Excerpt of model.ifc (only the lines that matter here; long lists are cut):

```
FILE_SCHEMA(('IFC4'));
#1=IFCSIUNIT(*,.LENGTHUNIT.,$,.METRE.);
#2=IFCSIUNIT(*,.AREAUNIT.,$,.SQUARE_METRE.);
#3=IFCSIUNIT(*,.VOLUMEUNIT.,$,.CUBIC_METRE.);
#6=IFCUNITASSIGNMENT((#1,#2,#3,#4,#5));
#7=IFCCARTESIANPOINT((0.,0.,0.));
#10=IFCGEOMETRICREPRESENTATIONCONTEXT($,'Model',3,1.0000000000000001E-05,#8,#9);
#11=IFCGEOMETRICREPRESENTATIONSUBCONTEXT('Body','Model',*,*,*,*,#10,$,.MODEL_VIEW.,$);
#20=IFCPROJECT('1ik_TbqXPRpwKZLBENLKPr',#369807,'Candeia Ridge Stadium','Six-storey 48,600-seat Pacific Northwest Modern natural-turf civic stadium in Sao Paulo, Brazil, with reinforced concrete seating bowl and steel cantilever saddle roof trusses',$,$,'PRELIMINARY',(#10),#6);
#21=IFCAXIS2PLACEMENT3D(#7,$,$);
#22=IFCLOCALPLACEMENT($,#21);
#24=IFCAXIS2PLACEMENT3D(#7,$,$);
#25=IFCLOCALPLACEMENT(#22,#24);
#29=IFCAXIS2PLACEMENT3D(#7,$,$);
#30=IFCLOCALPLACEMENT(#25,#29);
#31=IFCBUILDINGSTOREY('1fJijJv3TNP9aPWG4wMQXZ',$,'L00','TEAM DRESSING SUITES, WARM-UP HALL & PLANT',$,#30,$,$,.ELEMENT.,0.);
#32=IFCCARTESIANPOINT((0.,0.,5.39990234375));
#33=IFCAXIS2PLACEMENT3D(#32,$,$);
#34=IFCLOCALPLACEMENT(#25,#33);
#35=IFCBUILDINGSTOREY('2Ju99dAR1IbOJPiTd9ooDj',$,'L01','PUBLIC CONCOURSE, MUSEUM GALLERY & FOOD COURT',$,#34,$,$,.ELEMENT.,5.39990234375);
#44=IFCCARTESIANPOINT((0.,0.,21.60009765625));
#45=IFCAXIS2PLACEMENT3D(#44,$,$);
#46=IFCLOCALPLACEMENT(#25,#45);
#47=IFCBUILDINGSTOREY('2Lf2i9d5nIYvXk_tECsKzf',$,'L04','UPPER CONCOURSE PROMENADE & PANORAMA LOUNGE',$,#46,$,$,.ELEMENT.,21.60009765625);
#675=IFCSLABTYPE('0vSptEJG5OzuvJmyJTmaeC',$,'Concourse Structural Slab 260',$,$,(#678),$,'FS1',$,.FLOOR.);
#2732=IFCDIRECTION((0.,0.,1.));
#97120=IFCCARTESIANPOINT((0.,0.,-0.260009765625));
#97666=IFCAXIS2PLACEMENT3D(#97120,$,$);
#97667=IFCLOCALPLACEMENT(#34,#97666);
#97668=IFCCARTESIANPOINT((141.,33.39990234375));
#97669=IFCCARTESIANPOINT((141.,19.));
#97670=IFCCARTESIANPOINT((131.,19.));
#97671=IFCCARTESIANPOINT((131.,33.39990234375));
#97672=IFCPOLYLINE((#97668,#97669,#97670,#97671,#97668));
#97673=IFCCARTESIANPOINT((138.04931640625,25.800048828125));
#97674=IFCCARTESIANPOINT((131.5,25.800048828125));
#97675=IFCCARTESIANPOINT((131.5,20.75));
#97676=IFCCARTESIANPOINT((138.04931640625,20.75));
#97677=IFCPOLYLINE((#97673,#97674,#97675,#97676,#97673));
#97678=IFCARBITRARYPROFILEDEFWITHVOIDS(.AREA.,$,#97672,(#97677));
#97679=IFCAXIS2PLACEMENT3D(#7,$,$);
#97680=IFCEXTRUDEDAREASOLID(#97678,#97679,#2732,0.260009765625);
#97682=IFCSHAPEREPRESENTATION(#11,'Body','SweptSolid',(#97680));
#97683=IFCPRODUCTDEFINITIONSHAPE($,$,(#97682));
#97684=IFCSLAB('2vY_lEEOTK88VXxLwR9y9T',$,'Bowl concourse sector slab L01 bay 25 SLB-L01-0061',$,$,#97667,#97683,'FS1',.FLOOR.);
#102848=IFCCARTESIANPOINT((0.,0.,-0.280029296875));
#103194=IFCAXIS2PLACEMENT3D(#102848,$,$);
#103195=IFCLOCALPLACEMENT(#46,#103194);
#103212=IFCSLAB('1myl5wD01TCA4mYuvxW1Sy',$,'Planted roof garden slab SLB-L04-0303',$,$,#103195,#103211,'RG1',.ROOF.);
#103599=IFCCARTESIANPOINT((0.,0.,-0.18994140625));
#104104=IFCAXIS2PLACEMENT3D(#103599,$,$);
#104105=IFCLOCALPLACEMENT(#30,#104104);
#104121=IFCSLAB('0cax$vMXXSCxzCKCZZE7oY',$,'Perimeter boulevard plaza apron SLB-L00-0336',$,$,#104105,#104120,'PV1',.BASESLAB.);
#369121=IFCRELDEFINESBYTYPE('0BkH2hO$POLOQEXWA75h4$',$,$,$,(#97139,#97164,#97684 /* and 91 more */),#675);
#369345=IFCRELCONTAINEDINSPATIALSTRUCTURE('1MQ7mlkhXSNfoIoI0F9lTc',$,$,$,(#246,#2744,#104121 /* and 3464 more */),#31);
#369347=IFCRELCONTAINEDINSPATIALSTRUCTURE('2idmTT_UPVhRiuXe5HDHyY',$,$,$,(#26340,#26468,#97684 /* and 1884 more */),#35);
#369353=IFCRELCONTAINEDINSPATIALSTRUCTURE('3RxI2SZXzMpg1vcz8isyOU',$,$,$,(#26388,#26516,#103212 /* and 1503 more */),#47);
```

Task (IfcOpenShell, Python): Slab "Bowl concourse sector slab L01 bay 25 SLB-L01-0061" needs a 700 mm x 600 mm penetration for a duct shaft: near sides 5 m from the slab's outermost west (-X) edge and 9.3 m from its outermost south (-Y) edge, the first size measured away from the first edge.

```python
import numpy as np
import ifcopenshell
import ifcopenshell.api.feature
import ifcopenshell.api.geometry
import ifcopenshell.api.root
import ifcopenshell.geom
import ifcopenshell.util.placement
import ifcopenshell.util.representation
import ifcopenshell.util.shape
import ifcopenshell.util.unit

model = ifcopenshell.open("model.ifc")
unit_scale = ifcopenshell.util.unit.calculate_unit_scale(model)
settings = ifcopenshell.geom.settings()


def volume(element):
    """Net volume in cubic metres, openings subtracted."""
    shape = ifcopenshell.geom.create_shape(settings, element)
    return ifcopenshell.util.shape.get_volume(shape.geometry)


slab = model.by_guid("2vY_lEEOTK88VXxLwR9y9T")
before = volume(slab)

# Extent in the slab's own axes, in metres. The edges named are its -X and -Y sides.
slab_shape = ifcopenshell.geom.create_shape(settings, slab)
vertices = ifcopenshell.util.shape.get_vertices(slab_shape.geometry)
x_min, y_min, bottom = vertices.min(axis=0)
top = vertices[:, 2].max()

opening = ifcopenshell.api.root.create_entity(model, ifc_class="IfcOpeningElement", name="Duct shaft opening", predefined_type="OPENING")
context = ifcopenshell.util.representation.get_context(model, "Model", "Body", "MODEL_VIEW")
width, depth = 0.7, 0.6
outline = [(0.0, 0.0), (width, 0.0), (width, depth), (0.0, depth), (0.0, 0.0)]
# Overshoot both faces by 50 mm so the cut is clean.
shape = ifcopenshell.api.geometry.add_slab_representation(
    model, context=context, depth=top - bottom + 0.1, polyline=outline
)
ifcopenshell.api.geometry.assign_representation(model, product=opening, representation=shape)

matrix = ifcopenshell.util.placement.get_local_placement(slab.ObjectPlacement)
matrix[:, 3] = matrix @ np.append(np.array([x_min + 5, y_min + 9.3, bottom - 0.05]) / unit_scale, 1.0)
ifcopenshell.api.geometry.edit_object_placement(model, product=opening, matrix=matrix, is_si=False)
ifcopenshell.api.feature.add_feature(model, feature=opening, element=slab)

after = volume(slab)

print(f"slab volume {before:.3f} -> {after:.3f} m3")

model.write("model_edited.ifc")
```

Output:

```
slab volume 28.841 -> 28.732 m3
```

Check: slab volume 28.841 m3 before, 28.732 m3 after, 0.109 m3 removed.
